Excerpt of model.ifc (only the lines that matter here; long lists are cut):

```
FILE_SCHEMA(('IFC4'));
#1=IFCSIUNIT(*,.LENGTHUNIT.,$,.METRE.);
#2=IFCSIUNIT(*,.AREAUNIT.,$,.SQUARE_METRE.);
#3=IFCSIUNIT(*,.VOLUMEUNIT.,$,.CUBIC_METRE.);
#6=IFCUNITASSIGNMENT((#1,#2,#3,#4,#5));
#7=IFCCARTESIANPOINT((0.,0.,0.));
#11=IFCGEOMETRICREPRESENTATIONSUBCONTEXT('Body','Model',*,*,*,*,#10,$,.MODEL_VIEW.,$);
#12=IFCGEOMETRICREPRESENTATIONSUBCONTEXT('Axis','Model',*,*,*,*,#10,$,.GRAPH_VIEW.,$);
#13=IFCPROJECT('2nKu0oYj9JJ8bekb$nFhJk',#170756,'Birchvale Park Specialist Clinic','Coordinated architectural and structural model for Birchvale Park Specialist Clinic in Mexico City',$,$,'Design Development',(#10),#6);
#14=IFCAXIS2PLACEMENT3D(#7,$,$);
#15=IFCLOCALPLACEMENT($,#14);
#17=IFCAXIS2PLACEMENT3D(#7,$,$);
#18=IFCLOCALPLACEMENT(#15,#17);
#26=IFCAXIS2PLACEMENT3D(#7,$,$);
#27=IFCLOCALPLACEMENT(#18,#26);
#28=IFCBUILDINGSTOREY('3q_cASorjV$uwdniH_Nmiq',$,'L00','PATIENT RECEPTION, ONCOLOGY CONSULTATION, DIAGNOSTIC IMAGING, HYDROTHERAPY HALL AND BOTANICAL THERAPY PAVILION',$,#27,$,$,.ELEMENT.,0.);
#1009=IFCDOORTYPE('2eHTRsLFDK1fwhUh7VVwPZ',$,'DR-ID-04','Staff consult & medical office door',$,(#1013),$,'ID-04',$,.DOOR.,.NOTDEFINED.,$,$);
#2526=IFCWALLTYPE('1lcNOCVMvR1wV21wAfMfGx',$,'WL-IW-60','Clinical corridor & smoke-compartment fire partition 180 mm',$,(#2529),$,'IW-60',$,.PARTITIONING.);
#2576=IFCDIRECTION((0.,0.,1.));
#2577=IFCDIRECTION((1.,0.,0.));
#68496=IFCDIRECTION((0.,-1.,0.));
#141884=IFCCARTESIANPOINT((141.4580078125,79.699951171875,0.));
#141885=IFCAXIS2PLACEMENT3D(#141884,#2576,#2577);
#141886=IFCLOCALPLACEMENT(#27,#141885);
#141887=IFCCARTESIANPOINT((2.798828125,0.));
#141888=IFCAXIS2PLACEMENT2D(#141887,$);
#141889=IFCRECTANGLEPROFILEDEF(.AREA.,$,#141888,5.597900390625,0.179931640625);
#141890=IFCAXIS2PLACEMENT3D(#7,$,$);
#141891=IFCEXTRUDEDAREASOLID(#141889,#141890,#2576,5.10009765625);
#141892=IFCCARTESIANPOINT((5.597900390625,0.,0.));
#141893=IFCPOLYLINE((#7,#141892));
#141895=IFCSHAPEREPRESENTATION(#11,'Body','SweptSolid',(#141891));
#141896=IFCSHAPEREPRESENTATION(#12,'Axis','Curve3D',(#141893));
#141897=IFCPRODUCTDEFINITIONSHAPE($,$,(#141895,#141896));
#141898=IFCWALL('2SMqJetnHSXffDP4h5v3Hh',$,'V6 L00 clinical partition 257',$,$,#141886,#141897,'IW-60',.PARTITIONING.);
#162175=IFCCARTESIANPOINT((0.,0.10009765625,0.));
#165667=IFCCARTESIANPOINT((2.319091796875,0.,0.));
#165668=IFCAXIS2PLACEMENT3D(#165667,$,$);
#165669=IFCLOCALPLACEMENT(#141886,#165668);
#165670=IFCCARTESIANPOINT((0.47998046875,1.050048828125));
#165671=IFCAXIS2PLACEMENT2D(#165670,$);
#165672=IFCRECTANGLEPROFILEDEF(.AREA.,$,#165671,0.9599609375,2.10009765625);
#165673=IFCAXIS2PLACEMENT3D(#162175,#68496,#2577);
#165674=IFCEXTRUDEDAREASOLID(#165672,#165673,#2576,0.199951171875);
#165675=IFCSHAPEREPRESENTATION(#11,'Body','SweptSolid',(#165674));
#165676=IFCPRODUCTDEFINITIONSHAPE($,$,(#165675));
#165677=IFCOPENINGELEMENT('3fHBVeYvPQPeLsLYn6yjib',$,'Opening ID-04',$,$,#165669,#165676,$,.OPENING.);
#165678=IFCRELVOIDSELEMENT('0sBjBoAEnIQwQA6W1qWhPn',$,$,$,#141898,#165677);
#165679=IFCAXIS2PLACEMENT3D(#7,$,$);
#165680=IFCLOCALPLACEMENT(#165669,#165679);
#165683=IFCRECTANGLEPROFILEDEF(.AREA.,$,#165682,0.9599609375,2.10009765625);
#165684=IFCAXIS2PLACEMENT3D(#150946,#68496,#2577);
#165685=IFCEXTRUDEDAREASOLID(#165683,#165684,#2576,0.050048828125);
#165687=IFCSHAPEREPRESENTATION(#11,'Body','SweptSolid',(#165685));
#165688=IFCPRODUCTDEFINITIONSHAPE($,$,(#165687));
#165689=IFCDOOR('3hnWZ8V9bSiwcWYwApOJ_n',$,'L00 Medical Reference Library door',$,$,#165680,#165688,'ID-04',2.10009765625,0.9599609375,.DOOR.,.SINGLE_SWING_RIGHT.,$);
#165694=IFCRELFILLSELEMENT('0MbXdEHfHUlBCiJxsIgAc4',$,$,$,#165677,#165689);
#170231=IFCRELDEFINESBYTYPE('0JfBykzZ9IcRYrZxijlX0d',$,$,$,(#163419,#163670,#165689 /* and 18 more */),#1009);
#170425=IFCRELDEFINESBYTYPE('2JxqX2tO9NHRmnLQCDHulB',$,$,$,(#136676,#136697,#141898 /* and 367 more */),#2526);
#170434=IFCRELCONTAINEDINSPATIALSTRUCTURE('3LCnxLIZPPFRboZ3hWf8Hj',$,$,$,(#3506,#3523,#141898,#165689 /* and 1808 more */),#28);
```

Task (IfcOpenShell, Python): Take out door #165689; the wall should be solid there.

```python
import ifcopenshell
import ifcopenshell.api.feature
import ifcopenshell.api.root
import ifcopenshell.geom
import ifcopenshell.util.shape

model = ifcopenshell.open("model.ifc")
settings = ifcopenshell.geom.settings()


def volume(element):
    """Net volume in cubic metres, openings subtracted."""
    shape = ifcopenshell.geom.create_shape(settings, element)
    return ifcopenshell.util.shape.get_volume(shape.geometry)


door = model.by_id(165689)
opening = door.FillsVoids[0].RelatingOpeningElement
wall = opening.VoidsElements[0].RelatingBuildingElement
before = volume(wall)

ifcopenshell.api.root.remove_product(model, product=door)
ifcopenshell.api.feature.remove_feature(model, feature=opening)

after = volume(wall)

print(f"wall volume {before:.3f} -> {after:.3f} m3")

model.write("model_rev.ifc")
```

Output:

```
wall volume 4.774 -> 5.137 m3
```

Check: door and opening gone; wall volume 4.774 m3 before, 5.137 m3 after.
